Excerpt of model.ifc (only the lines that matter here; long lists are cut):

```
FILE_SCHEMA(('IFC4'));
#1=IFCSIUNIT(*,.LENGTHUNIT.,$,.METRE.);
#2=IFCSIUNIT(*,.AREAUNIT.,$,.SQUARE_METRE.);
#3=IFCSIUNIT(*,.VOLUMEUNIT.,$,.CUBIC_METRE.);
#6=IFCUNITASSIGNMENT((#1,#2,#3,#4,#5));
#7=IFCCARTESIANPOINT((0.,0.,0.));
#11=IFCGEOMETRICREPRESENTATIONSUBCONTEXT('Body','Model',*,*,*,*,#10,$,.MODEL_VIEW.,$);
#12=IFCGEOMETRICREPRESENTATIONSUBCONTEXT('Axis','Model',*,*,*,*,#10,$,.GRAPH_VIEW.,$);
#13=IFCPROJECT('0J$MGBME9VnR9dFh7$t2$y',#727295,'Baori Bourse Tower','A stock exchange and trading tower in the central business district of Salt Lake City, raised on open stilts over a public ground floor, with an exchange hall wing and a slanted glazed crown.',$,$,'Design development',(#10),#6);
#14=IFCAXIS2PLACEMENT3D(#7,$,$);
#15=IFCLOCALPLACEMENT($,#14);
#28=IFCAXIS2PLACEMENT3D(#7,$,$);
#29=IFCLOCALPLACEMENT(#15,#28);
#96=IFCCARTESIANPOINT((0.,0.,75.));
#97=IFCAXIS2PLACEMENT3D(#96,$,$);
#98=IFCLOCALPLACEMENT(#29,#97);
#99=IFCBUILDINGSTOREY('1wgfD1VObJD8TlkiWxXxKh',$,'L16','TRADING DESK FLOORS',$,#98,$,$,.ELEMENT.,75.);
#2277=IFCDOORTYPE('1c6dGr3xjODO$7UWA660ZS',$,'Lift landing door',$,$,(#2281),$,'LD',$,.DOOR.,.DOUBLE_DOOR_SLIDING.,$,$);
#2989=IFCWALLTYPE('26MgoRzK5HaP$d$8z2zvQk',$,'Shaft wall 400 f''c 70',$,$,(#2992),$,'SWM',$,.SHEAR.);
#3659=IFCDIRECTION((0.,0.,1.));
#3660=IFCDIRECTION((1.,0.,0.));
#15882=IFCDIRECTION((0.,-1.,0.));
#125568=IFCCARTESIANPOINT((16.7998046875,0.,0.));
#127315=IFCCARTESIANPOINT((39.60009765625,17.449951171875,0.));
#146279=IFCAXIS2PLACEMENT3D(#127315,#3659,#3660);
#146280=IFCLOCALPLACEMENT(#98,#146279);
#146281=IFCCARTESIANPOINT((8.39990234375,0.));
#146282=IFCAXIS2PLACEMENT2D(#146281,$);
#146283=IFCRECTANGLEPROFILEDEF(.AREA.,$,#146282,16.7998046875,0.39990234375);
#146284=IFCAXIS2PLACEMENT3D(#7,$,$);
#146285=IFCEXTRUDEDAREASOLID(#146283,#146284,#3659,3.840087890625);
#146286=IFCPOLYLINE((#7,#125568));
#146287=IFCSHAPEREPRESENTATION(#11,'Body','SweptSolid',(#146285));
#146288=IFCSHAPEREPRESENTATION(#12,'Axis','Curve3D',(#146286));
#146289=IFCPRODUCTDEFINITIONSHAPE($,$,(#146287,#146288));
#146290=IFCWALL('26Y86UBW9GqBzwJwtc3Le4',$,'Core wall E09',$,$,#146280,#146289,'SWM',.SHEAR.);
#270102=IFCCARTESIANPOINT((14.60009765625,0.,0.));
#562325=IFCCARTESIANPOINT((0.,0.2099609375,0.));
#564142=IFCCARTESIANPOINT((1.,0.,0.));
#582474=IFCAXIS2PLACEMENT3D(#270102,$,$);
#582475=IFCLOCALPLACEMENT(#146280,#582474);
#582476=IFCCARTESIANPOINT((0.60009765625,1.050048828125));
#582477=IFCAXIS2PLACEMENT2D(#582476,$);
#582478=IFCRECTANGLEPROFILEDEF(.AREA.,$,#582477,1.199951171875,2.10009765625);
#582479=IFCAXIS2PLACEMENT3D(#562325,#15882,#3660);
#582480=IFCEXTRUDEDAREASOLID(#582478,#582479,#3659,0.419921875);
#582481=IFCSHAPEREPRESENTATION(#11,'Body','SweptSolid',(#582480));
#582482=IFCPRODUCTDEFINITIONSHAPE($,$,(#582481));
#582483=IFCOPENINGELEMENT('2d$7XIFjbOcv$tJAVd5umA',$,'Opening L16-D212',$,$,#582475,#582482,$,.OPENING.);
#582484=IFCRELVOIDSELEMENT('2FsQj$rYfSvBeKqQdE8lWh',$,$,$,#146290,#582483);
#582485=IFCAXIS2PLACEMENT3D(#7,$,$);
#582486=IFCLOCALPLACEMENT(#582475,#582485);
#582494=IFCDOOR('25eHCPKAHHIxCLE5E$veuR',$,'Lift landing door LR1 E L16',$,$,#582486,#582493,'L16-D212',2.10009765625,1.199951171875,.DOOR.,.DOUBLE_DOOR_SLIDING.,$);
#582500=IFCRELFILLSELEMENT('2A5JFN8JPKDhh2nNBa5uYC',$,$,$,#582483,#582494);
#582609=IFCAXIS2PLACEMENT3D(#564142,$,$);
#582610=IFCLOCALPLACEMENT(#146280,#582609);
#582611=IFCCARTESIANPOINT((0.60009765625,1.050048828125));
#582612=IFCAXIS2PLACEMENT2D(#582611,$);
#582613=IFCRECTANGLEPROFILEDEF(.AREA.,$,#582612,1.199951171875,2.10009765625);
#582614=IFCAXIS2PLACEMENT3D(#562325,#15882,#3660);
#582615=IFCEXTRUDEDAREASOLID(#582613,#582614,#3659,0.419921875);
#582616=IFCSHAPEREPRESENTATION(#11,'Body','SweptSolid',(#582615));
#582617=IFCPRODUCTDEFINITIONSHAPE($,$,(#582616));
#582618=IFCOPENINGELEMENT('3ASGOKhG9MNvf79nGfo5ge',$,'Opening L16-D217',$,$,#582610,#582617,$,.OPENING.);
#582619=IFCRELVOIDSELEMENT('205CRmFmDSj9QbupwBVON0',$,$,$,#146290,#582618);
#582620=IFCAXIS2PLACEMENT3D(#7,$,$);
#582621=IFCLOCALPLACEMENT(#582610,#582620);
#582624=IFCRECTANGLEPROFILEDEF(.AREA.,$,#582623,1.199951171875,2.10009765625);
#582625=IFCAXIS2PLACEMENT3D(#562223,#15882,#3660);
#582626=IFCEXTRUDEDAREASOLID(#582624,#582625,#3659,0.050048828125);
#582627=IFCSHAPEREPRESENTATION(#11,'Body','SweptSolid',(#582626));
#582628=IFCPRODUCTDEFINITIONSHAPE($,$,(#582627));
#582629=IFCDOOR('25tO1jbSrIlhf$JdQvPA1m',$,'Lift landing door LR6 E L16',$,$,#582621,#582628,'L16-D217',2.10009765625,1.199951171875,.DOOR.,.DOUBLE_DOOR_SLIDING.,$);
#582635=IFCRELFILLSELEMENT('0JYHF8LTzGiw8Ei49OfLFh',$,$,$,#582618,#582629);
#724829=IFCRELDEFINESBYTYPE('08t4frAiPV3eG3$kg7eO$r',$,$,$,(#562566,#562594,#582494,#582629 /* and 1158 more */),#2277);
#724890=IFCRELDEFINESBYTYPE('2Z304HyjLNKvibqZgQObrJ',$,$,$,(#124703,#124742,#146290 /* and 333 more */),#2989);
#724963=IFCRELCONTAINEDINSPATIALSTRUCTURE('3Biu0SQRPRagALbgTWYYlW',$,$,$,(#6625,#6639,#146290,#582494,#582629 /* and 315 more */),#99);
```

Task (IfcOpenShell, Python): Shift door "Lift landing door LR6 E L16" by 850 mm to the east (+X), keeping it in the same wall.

```python
import ifcopenshell
import ifcopenshell.api.geometry
import ifcopenshell.util.placement
import ifcopenshell.util.unit

model = ifcopenshell.open("model.ifc")
unit_scale = ifcopenshell.util.unit.calculate_unit_scale(model)

door = model.by_guid("25tO1jbSrIlhf$JdQvPA1m")
opening = door.FillsVoids[0].RelatingOpeningElement
wall = opening.VoidsElements[0].RelatingBuildingElement

wall_matrix = ifcopenshell.util.placement.get_local_placement(wall.ObjectPlacement)
shift = wall_matrix[:3, 0] * 0.85 / unit_scale
before = ifcopenshell.util.placement.get_local_placement(door.ObjectPlacement)[:3, 3].copy()

# The door is placed relative to its opening, so it follows when the opening moves.
matrix = ifcopenshell.util.placement.get_local_placement(opening.ObjectPlacement)
matrix[:3, 3] += shift
ifcopenshell.api.geometry.edit_object_placement(
    model, product=opening, matrix=matrix, is_si=False, should_transform_children=True
)

after = ifcopenshell.util.placement.get_local_placement(door.ObjectPlacement)[:3, 3]
print("door moved by", (after - before).round(3) + 0.0)

model.write("model_edited.ifc")
```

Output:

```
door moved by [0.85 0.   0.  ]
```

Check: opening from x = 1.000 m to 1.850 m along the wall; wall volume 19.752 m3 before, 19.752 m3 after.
